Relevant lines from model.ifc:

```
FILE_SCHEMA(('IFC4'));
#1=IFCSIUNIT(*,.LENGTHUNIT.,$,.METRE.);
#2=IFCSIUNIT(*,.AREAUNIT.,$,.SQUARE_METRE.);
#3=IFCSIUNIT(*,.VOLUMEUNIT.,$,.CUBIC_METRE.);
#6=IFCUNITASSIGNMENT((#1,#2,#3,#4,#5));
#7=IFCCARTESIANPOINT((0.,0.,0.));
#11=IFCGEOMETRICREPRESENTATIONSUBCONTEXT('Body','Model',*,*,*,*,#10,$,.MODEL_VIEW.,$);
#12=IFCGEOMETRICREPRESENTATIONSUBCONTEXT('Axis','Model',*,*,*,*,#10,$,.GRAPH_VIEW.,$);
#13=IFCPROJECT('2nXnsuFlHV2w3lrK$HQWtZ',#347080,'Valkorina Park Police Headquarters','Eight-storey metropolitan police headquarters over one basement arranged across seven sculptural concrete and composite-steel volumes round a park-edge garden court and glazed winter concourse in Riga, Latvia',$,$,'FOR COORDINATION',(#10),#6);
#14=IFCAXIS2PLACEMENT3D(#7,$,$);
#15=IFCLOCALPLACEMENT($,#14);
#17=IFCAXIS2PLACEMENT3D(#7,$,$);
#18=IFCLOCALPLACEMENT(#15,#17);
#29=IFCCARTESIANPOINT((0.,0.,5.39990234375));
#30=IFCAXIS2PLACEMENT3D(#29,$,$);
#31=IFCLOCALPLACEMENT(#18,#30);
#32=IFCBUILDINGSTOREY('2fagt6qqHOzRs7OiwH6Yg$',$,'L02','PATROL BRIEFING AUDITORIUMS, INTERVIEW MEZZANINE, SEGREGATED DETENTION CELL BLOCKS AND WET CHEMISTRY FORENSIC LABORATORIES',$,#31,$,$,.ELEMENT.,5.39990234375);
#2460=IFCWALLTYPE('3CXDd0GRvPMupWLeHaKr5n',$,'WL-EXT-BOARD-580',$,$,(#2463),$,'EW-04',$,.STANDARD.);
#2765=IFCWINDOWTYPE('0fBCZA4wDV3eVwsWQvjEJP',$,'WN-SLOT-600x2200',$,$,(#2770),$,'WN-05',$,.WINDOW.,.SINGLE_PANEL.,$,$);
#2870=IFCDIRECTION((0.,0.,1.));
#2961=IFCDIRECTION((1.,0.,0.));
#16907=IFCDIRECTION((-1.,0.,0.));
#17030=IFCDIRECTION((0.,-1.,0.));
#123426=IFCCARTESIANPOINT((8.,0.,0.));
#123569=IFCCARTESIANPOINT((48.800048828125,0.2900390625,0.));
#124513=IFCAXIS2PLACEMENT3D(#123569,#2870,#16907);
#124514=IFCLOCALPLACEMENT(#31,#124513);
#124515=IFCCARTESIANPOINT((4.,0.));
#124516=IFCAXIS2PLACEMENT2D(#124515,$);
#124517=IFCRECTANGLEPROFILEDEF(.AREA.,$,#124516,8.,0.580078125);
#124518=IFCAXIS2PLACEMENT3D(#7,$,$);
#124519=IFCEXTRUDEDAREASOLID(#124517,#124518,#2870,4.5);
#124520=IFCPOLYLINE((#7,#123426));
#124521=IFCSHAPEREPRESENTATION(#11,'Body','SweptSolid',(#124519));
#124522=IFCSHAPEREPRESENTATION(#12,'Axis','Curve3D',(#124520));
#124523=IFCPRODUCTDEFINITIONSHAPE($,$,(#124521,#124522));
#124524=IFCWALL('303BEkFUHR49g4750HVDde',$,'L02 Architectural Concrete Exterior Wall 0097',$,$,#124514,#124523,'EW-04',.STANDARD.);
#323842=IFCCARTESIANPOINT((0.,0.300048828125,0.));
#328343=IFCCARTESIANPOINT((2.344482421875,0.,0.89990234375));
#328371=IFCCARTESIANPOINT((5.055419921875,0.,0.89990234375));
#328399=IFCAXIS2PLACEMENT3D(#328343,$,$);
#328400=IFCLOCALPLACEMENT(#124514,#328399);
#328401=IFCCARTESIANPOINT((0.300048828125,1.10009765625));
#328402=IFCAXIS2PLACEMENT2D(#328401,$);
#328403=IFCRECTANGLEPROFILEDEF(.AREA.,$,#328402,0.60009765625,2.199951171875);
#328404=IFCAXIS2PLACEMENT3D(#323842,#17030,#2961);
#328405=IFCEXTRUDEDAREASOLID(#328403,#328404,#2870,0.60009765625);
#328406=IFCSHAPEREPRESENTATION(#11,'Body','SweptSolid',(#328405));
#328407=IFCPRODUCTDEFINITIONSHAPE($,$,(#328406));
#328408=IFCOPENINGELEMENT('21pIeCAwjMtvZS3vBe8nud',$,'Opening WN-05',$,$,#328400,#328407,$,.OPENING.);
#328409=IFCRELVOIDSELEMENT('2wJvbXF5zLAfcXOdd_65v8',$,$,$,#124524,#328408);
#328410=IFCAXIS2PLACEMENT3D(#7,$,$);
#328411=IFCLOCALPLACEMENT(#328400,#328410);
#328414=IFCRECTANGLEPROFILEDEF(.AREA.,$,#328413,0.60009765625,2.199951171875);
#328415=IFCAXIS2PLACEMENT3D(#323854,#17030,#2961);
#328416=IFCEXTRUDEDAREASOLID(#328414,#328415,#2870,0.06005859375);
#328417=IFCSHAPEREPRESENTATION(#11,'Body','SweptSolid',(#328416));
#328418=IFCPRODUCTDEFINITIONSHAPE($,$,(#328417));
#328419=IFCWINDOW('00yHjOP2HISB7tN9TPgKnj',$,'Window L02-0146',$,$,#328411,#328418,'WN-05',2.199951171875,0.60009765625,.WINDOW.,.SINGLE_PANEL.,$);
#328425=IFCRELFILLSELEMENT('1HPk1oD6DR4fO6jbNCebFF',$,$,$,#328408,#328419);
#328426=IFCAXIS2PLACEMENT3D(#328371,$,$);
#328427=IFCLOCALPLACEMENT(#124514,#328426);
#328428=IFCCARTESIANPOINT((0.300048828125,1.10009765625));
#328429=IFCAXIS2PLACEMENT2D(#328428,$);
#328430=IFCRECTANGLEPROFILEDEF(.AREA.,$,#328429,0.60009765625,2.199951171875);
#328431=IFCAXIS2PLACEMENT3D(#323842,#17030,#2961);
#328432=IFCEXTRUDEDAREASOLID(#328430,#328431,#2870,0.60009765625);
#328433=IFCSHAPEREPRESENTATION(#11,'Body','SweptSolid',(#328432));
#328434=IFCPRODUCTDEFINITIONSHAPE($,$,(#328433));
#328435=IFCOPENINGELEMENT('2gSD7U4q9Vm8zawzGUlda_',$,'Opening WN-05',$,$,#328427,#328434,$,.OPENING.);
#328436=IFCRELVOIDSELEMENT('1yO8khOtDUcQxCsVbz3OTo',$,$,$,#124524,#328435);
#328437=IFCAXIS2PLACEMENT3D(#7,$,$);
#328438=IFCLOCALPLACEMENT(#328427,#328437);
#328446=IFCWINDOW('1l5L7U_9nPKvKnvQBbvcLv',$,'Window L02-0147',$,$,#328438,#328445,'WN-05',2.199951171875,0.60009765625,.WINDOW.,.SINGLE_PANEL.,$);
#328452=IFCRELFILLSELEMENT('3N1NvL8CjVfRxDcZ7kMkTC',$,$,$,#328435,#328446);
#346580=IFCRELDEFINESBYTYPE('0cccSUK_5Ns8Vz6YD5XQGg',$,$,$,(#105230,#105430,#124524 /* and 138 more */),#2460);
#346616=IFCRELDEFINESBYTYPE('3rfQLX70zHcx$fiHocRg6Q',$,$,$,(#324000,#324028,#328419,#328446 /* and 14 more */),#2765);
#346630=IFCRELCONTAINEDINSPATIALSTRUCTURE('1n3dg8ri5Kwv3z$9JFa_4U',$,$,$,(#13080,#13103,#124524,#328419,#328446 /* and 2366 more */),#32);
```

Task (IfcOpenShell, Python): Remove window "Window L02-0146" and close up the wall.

```python
import ifcopenshell
import ifcopenshell.api.feature
import ifcopenshell.api.root
import ifcopenshell.geom
import ifcopenshell.util.shape

model = ifcopenshell.open("model.ifc")
settings = ifcopenshell.geom.settings()


def volume(element):
    """Net volume in cubic metres, openings subtracted."""
    shape = ifcopenshell.geom.create_shape(settings, element)
    return ifcopenshell.util.shape.get_volume(shape.geometry)


window = model.by_id(328419)
opening = window.FillsVoids[0].RelatingOpeningElement
wall = opening.VoidsElements[0].RelatingBuildingElement
before = volume(wall)

ifcopenshell.api.root.remove_product(model, product=window)
ifcopenshell.api.feature.remove_feature(model, feature=opening)

after = volume(wall)

print(f"wall volume {before:.3f} -> {after:.3f} m3")

model.write("model_v2.ifc")
```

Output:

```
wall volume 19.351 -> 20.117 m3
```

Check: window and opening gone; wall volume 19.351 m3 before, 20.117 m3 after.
